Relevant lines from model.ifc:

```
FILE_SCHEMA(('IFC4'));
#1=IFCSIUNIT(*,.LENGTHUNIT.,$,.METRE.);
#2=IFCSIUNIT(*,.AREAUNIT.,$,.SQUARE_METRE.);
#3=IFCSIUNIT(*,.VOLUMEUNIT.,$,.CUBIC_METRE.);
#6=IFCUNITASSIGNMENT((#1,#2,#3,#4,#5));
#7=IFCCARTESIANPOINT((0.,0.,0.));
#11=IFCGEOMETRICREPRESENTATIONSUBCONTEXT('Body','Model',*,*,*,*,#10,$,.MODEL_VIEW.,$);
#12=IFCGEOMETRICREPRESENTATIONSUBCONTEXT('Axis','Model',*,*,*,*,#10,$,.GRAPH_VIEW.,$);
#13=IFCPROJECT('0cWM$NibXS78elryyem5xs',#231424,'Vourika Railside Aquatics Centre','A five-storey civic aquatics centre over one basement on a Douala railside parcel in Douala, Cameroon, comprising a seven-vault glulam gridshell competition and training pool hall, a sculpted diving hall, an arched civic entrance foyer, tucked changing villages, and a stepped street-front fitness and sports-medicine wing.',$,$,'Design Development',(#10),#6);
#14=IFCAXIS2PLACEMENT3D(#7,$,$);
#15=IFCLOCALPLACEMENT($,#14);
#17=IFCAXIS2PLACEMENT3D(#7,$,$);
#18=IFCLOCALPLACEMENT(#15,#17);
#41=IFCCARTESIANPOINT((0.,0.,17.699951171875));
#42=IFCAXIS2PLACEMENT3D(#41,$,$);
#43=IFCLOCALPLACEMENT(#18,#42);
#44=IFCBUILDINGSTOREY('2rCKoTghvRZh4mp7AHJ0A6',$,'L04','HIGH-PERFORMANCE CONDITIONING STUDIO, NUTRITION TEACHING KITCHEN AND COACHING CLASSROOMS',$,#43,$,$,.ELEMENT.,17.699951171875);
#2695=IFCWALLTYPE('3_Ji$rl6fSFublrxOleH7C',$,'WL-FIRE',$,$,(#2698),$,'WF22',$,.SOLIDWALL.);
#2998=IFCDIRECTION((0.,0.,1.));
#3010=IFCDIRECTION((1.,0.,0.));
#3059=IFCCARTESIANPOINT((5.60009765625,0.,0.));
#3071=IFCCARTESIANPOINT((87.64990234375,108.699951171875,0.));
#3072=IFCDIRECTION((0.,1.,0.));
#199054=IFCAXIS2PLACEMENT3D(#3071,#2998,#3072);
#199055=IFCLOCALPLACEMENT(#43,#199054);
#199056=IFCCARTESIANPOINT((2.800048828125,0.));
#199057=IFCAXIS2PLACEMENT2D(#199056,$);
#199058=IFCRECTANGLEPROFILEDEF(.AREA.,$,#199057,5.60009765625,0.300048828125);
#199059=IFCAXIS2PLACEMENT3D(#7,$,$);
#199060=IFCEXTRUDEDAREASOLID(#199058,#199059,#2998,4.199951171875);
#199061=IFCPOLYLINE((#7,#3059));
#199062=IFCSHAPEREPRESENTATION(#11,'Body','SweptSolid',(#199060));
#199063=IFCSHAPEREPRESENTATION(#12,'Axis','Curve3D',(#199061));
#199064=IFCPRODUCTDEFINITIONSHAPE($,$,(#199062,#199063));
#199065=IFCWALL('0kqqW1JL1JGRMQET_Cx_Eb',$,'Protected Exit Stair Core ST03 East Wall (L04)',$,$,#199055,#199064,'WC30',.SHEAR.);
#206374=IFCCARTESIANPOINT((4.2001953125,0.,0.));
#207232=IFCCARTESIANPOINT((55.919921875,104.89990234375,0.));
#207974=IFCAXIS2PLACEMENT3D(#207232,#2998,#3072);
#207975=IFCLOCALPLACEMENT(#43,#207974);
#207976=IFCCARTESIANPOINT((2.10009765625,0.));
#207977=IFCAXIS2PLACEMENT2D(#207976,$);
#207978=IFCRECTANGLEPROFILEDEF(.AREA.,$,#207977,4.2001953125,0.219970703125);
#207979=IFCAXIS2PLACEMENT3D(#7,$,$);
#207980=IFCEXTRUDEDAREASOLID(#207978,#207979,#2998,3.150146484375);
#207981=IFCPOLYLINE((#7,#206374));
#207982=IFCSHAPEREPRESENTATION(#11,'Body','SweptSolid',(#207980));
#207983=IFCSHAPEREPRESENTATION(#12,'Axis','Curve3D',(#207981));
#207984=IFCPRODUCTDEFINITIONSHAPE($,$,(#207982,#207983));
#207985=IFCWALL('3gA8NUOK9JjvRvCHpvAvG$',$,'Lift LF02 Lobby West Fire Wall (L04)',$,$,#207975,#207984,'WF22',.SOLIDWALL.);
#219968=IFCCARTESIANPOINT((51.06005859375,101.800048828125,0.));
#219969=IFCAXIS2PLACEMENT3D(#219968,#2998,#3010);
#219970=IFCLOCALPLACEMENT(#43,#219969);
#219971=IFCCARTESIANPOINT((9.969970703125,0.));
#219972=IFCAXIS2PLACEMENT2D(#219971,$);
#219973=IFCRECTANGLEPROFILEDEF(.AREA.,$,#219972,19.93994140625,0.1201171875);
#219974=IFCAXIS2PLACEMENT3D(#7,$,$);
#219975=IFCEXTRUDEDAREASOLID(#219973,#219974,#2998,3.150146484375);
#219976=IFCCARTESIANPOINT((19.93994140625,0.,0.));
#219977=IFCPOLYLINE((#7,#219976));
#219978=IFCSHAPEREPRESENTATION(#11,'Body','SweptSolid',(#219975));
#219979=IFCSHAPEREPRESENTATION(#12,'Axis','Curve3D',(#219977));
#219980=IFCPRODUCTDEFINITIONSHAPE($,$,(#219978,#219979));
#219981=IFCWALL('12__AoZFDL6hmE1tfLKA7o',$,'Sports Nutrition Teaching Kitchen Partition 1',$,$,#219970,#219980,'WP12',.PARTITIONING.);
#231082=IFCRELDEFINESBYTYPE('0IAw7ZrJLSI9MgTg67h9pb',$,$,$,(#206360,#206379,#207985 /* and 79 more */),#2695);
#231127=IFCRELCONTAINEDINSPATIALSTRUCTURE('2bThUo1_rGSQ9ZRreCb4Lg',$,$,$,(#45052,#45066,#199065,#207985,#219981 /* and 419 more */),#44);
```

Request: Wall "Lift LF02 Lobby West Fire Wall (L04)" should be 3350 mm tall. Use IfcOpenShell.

```python
import ifcopenshell
import ifcopenshell.geom
import ifcopenshell.util.representation
import ifcopenshell.util.shape
import ifcopenshell.util.unit

model = ifcopenshell.open("model.ifc")
unit_scale = ifcopenshell.util.unit.calculate_unit_scale(model)
settings = ifcopenshell.geom.settings()


def volume(element):
    """Net volume in cubic metres, openings subtracted."""
    shape = ifcopenshell.geom.create_shape(settings, element)
    return ifcopenshell.util.shape.get_volume(shape.geometry)


wall = model.by_guid("3gA8NUOK9JjvRvCHpvAvG$")
before = volume(wall)

body = ifcopenshell.util.representation.get_representation(wall, "Model", "Body")
solid = body.Items[0]
old_height = solid.Depth
solid.Depth = 3.35 / unit_scale
after = volume(wall)

print(f"height {old_height:g} -> {solid.Depth:g}, volume {before:.3f} -> {after:.3f} m3")

model.write("model_edited.ifc")
```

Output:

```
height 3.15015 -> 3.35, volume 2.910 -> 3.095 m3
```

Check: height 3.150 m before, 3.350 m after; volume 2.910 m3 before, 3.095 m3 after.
